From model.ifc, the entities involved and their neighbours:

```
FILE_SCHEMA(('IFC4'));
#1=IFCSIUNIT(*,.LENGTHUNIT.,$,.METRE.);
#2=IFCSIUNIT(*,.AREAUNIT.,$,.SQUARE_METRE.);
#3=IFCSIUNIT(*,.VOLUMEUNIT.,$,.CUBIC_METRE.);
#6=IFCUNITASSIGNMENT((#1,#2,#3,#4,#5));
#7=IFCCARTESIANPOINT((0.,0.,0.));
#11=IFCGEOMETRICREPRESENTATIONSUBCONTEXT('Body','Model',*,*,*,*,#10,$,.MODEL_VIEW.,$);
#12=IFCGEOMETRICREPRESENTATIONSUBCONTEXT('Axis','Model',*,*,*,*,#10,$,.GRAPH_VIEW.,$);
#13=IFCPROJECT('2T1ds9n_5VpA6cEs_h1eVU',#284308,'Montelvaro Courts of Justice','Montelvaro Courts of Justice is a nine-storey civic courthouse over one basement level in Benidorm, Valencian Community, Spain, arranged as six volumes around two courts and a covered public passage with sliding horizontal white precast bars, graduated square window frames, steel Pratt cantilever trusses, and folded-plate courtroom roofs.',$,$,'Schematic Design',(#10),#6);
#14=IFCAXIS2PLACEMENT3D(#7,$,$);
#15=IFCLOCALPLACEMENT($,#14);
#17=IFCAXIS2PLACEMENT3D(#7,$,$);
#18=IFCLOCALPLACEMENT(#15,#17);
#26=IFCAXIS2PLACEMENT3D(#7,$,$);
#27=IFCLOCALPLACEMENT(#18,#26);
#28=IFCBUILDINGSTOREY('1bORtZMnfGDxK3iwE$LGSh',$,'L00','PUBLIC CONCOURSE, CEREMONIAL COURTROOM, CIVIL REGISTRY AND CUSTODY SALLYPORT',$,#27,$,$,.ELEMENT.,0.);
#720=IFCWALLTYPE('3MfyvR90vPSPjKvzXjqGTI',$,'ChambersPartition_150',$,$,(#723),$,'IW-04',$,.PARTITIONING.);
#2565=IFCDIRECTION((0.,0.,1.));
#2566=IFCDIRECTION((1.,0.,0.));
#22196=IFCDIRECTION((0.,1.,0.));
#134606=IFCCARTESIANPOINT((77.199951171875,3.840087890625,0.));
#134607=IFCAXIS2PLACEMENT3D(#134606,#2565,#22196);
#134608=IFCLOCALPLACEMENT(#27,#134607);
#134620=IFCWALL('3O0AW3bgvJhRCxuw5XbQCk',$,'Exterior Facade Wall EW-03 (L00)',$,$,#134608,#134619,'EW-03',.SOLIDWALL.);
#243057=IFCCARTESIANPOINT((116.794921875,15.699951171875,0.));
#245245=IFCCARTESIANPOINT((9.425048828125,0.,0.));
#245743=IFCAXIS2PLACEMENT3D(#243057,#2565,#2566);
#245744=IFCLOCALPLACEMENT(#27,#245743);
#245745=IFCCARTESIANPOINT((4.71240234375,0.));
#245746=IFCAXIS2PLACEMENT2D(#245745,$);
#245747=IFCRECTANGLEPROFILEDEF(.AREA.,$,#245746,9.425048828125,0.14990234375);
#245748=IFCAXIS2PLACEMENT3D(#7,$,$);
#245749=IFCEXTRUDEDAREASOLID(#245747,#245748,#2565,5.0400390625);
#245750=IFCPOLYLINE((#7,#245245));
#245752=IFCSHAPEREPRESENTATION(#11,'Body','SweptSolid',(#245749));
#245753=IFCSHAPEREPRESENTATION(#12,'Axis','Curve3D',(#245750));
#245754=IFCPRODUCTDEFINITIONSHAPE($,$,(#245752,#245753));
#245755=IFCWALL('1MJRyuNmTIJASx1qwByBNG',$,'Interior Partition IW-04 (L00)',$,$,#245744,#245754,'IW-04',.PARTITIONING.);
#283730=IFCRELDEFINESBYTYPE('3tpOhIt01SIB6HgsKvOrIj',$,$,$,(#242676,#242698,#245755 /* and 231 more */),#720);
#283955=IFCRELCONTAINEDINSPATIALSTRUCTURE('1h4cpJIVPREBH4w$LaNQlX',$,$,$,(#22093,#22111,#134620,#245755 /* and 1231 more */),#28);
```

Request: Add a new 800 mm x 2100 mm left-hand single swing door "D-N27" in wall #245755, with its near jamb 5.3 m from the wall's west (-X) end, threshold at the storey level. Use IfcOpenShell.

```python
import numpy as np
import ifcopenshell
import ifcopenshell.api.feature
import ifcopenshell.api.geometry
import ifcopenshell.api.root
import ifcopenshell.api.spatial
import ifcopenshell.geom
import ifcopenshell.util.element
import ifcopenshell.util.placement
import ifcopenshell.util.representation
import ifcopenshell.util.shape
import ifcopenshell.util.unit

model = ifcopenshell.open("model.ifc")
unit_scale = ifcopenshell.util.unit.calculate_unit_scale(model)
settings = ifcopenshell.geom.settings()


def volume(element):
    """Net volume in cubic metres, openings subtracted."""
    shape = ifcopenshell.geom.create_shape(settings, element)
    return ifcopenshell.util.shape.get_volume(shape.geometry)


wall = model.by_guid("1MJRyuNmTIJASx1qwByBNG")
storey = ifcopenshell.util.element.get_container(wall, ifc_class="IfcBuildingStorey")
context = ifcopenshell.util.representation.get_context(model, "Model", "Body", "MODEL_VIEW")
before = volume(wall)

width, height, from_end, sill = 0.8, 2.1, 5.3, 0.0  # metres

# The wall runs along its own X axis, and the end named is its -X end.
wall_shape = ifcopenshell.geom.create_shape(settings, wall)
x, y, z = ifcopenshell.util.shape.get_vertices(wall_shape.geometry).T
start = x.min() + from_end
face, thickness = float(y.min()), float(y.max() - y.min())
wall_matrix = ifcopenshell.util.placement.get_local_placement(wall.ObjectPlacement)
level = ifcopenshell.util.placement.get_local_placement(storey.ObjectPlacement)[2, 3]


def in_wall(x, y):
    """Placement at x, y metres in the wall's axes, at sill height."""
    matrix = wall_matrix.copy()
    matrix[:, 3] = wall_matrix @ np.array([x / unit_scale, y / unit_scale, 0.0, 1.0])
    matrix[2, 3] = level + sill / unit_scale
    return matrix


# Opening: a box that overshoots both wall faces by 50 mm.
opening = ifcopenshell.api.root.create_entity(model, ifc_class="IfcOpeningElement", predefined_type="OPENING")
box = ifcopenshell.api.geometry.add_wall_representation(
    model, context=context, length=width, height=height, thickness=thickness + 0.1
)
ifcopenshell.api.geometry.assign_representation(model, product=opening, representation=box)
ifcopenshell.api.geometry.edit_object_placement(model, product=opening, matrix=in_wall(start, face - 0.05), is_si=False)
ifcopenshell.api.feature.add_feature(model, feature=opening, element=wall)

door = ifcopenshell.api.root.create_entity(model, ifc_class="IfcDoor", name="D-N27", predefined_type="DOOR")
door.OverallWidth, door.OverallHeight = width / unit_scale, height / unit_scale
door.OperationType = "SINGLE_SWING_LEFT"
body = ifcopenshell.api.geometry.add_door_representation(
    model,
    context=context,
    overall_width=door.OverallWidth,
    overall_height=door.OverallHeight,
    operation_type="SINGLE_SWING_LEFT",
    lining_properties={"LiningDepth": thickness / unit_scale, "ThresholdDepth": thickness / unit_scale},
)
ifcopenshell.api.geometry.assign_representation(model, product=door, representation=body)
ifcopenshell.api.spatial.assign_container(model, products=[door], relating_structure=storey)
ifcopenshell.api.feature.add_filling(model, opening=opening, element=door)

# The lining spans the wall, so the door starts at the wall face.
ifcopenshell.api.geometry.edit_object_placement(model, product=door, matrix=in_wall(start, face), is_si=False)

after = volume(wall)

print(f"wall volume {before:.3f} -> {after:.3f} m3")

model.write("model_edited.ifc")
```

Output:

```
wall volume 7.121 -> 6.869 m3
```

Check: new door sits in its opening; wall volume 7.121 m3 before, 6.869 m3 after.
